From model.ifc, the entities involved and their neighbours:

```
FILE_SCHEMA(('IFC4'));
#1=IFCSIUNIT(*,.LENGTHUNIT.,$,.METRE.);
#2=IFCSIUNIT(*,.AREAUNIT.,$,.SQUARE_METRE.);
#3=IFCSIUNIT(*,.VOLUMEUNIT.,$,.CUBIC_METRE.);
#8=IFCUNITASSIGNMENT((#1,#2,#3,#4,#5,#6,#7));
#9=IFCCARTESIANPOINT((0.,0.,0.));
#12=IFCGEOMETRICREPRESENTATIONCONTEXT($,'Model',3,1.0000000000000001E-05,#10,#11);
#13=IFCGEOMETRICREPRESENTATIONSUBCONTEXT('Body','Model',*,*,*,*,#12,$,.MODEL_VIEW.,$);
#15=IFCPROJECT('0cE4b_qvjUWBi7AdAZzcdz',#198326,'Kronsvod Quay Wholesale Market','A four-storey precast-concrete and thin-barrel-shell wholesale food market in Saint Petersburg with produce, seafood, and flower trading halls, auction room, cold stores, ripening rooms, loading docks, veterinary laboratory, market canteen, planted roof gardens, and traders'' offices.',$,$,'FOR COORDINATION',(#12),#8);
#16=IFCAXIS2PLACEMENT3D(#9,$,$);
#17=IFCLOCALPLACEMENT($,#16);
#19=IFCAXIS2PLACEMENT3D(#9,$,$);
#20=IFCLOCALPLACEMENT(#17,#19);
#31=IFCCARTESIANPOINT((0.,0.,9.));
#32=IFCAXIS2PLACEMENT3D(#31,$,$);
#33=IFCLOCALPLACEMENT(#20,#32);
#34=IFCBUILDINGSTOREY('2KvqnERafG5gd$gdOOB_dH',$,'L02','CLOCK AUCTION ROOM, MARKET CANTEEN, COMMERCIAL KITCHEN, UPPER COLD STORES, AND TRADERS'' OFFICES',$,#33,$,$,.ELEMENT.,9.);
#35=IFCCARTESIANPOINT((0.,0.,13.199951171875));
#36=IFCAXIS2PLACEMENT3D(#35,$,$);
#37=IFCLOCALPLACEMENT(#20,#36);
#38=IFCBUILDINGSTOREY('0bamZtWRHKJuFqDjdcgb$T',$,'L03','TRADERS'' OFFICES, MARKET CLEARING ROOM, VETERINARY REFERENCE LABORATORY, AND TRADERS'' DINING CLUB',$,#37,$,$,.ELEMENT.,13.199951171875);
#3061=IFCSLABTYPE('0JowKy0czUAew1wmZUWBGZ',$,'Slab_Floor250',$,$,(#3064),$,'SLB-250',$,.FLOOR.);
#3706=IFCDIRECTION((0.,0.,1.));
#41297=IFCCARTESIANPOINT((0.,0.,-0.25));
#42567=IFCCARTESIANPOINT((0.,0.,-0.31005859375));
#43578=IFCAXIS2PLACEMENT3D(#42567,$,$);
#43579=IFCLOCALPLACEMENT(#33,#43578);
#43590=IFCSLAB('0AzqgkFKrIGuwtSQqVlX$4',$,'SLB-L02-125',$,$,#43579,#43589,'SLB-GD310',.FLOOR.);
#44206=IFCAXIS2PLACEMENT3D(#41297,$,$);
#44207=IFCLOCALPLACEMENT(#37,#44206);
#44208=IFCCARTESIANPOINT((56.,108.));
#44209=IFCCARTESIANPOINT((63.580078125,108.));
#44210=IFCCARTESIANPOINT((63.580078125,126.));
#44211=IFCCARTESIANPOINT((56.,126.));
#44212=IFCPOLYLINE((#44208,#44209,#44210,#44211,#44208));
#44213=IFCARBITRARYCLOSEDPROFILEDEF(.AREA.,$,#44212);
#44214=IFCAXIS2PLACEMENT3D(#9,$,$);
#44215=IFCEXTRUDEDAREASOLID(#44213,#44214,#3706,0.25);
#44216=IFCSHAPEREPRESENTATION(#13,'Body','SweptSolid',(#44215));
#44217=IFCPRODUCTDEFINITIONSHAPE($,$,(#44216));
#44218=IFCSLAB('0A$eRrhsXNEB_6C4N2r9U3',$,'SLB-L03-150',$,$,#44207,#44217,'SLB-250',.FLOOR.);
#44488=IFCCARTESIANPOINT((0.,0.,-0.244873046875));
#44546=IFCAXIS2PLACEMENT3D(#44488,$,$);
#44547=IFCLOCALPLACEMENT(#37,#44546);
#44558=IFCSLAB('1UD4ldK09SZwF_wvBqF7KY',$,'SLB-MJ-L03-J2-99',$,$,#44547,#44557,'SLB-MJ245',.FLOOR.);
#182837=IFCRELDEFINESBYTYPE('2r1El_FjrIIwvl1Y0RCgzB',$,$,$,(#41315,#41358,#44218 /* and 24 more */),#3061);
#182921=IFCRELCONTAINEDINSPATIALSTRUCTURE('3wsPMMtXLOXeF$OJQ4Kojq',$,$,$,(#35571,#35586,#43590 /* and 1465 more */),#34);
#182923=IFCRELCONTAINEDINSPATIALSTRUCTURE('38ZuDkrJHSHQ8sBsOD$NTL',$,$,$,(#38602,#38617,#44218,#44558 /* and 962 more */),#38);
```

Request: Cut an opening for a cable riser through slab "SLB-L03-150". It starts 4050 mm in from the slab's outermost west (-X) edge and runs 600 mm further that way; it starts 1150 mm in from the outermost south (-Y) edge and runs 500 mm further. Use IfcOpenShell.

```python
import numpy as np
import ifcopenshell
import ifcopenshell.api.feature
import ifcopenshell.api.geometry
import ifcopenshell.api.root
import ifcopenshell.geom
import ifcopenshell.util.placement
import ifcopenshell.util.representation
import ifcopenshell.util.shape
import ifcopenshell.util.unit

model = ifcopenshell.open("model.ifc")
unit_scale = ifcopenshell.util.unit.calculate_unit_scale(model)
settings = ifcopenshell.geom.settings()


def volume(element):
    """Net volume in cubic metres, openings subtracted."""
    shape = ifcopenshell.geom.create_shape(settings, element)
    return ifcopenshell.util.shape.get_volume(shape.geometry)


slab = model.by_guid("0A$eRrhsXNEB_6C4N2r9U3")
before = volume(slab)

# Extent in the slab's own axes, in metres. The edges named are its -X and -Y sides.
slab_shape = ifcopenshell.geom.create_shape(settings, slab)
vertices = ifcopenshell.util.shape.get_vertices(slab_shape.geometry)
x_min, y_min, bottom = vertices.min(axis=0)
top = vertices[:, 2].max()

opening = ifcopenshell.api.root.create_entity(model, ifc_class="IfcOpeningElement", name="Cable riser opening", predefined_type="OPENING")
context = ifcopenshell.util.representation.get_context(model, "Model", "Body", "MODEL_VIEW")
width, depth = 0.6, 0.5
outline = [(0.0, 0.0), (width, 0.0), (width, depth), (0.0, depth), (0.0, 0.0)]
# Overshoot both faces by 50 mm so the cut is clean.
shape = ifcopenshell.api.geometry.add_slab_representation(
    model, context=context, depth=top - bottom + 0.1, polyline=outline
)
ifcopenshell.api.geometry.assign_representation(model, product=opening, representation=shape)

matrix = ifcopenshell.util.placement.get_local_placement(slab.ObjectPlacement)
matrix[:, 3] = matrix @ np.append(np.array([x_min + 4.05, y_min + 1.15, bottom - 0.05]) / unit_scale, 1.0)
ifcopenshell.api.geometry.edit_object_placement(model, product=opening, matrix=matrix, is_si=False)
ifcopenshell.api.feature.add_feature(model, feature=opening, element=slab)

after = volume(slab)

print(f"slab volume {before:.3f} -> {after:.3f} m3")

model.write("model-out.ifc")
```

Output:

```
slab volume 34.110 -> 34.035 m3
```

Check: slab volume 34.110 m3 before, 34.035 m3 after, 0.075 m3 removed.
